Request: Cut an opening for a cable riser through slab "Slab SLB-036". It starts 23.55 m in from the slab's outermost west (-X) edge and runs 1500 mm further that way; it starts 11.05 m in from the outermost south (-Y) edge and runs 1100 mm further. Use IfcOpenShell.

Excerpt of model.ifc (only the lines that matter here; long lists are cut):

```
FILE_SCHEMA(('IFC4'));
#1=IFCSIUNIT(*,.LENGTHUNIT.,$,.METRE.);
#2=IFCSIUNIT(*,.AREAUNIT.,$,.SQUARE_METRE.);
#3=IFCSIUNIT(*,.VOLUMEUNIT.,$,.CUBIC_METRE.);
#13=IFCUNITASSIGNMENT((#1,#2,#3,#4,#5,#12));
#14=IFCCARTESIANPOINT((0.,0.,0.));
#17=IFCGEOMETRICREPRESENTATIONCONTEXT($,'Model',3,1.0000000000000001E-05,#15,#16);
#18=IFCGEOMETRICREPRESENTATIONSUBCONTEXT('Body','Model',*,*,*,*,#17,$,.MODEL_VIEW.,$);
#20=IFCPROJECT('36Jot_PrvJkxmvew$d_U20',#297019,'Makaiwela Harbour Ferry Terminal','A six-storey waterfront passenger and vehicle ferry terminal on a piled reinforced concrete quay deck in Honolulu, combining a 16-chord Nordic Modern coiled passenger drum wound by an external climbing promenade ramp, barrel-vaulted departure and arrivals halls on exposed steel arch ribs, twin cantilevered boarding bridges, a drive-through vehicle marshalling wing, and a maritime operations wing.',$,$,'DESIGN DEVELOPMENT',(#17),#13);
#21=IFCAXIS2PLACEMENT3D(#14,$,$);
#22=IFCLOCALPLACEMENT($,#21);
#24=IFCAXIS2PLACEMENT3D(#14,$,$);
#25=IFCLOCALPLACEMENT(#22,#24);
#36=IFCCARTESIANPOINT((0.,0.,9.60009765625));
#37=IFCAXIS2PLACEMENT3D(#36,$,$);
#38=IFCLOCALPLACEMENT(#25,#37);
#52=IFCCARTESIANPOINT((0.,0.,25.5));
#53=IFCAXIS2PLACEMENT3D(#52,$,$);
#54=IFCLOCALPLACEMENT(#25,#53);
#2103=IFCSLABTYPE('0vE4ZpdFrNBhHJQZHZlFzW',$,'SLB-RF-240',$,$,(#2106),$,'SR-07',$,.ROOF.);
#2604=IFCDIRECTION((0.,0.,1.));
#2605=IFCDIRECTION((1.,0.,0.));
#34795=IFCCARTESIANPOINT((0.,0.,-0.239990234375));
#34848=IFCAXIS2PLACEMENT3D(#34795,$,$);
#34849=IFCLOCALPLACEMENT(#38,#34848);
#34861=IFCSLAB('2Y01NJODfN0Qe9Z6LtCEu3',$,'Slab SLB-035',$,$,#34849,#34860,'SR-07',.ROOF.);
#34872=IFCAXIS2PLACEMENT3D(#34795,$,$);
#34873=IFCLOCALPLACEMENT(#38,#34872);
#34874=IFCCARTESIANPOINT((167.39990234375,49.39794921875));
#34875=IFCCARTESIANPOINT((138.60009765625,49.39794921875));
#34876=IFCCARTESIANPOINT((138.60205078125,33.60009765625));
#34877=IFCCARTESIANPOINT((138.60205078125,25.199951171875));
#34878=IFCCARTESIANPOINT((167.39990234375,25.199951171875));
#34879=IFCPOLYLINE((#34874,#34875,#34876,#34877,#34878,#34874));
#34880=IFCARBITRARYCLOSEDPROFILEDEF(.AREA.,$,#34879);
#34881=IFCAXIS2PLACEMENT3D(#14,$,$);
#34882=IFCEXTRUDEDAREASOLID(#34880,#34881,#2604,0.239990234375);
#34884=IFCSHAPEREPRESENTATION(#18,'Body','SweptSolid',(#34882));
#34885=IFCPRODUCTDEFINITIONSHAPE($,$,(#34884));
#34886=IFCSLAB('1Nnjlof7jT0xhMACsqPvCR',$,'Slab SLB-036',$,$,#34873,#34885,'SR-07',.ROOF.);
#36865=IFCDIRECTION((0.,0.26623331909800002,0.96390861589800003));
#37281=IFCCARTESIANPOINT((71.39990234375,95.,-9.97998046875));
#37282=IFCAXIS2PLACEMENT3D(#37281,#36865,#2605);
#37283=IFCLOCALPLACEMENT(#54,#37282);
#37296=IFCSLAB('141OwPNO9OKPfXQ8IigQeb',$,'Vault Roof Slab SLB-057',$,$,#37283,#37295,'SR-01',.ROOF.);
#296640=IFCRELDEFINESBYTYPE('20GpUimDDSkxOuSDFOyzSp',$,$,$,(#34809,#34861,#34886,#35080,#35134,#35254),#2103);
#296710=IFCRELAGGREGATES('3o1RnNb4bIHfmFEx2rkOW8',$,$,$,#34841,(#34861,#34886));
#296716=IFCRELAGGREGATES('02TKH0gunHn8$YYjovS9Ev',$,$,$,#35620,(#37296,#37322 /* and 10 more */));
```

```python
import numpy as np
import ifcopenshell
import ifcopenshell.api.feature
import ifcopenshell.api.geometry
import ifcopenshell.api.root
import ifcopenshell.geom
import ifcopenshell.util.placement
import ifcopenshell.util.representation
import ifcopenshell.util.shape
import ifcopenshell.util.unit

model = ifcopenshell.open("model.ifc")
unit_scale = ifcopenshell.util.unit.calculate_unit_scale(model)
settings = ifcopenshell.geom.settings()


def volume(element):
    """Net volume in cubic metres, openings subtracted."""
    shape = ifcopenshell.geom.create_shape(settings, element)
    return ifcopenshell.util.shape.get_volume(shape.geometry)


slab = model.by_guid("1Nnjlof7jT0xhMACsqPvCR")
before = volume(slab)

# Extent in the slab's own axes, in metres. The edges named are its -X and -Y sides.
slab_shape = ifcopenshell.geom.create_shape(settings, slab)
vertices = ifcopenshell.util.shape.get_vertices(slab_shape.geometry)
x_min, y_min, bottom = vertices.min(axis=0)
top = vertices[:, 2].max()

opening = ifcopenshell.api.root.create_entity(model, ifc_class="IfcOpeningElement", name="Cable riser opening", predefined_type="OPENING")
context = ifcopenshell.util.representation.get_context(model, "Model", "Body", "MODEL_VIEW")
width, depth = 1.5, 1.1
outline = [(0.0, 0.0), (width, 0.0), (width, depth), (0.0, depth), (0.0, 0.0)]
# Overshoot both faces by 50 mm so the cut is clean.
shape = ifcopenshell.api.geometry.add_slab_representation(
    model, context=context, depth=top - bottom + 0.1, polyline=outline
)
ifcopenshell.api.geometry.assign_representation(model, product=opening, representation=shape)

matrix = ifcopenshell.util.placement.get_local_placement(slab.ObjectPlacement)
matrix[:, 3] = matrix @ np.append(np.array([x_min + 23.55, y_min + 11.05, bottom - 0.05]) / unit_scale, 1.0)
ifcopenshell.api.geometry.edit_object_placement(model, product=opening, matrix=matrix, is_si=False)
ifcopenshell.api.feature.add_feature(model, feature=opening, element=slab)

after = volume(slab)

print(f"slab volume {before:.3f} -> {after:.3f} m3")

model.write("model-out.ifc")
```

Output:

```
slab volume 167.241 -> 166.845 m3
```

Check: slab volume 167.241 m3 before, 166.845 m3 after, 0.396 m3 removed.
